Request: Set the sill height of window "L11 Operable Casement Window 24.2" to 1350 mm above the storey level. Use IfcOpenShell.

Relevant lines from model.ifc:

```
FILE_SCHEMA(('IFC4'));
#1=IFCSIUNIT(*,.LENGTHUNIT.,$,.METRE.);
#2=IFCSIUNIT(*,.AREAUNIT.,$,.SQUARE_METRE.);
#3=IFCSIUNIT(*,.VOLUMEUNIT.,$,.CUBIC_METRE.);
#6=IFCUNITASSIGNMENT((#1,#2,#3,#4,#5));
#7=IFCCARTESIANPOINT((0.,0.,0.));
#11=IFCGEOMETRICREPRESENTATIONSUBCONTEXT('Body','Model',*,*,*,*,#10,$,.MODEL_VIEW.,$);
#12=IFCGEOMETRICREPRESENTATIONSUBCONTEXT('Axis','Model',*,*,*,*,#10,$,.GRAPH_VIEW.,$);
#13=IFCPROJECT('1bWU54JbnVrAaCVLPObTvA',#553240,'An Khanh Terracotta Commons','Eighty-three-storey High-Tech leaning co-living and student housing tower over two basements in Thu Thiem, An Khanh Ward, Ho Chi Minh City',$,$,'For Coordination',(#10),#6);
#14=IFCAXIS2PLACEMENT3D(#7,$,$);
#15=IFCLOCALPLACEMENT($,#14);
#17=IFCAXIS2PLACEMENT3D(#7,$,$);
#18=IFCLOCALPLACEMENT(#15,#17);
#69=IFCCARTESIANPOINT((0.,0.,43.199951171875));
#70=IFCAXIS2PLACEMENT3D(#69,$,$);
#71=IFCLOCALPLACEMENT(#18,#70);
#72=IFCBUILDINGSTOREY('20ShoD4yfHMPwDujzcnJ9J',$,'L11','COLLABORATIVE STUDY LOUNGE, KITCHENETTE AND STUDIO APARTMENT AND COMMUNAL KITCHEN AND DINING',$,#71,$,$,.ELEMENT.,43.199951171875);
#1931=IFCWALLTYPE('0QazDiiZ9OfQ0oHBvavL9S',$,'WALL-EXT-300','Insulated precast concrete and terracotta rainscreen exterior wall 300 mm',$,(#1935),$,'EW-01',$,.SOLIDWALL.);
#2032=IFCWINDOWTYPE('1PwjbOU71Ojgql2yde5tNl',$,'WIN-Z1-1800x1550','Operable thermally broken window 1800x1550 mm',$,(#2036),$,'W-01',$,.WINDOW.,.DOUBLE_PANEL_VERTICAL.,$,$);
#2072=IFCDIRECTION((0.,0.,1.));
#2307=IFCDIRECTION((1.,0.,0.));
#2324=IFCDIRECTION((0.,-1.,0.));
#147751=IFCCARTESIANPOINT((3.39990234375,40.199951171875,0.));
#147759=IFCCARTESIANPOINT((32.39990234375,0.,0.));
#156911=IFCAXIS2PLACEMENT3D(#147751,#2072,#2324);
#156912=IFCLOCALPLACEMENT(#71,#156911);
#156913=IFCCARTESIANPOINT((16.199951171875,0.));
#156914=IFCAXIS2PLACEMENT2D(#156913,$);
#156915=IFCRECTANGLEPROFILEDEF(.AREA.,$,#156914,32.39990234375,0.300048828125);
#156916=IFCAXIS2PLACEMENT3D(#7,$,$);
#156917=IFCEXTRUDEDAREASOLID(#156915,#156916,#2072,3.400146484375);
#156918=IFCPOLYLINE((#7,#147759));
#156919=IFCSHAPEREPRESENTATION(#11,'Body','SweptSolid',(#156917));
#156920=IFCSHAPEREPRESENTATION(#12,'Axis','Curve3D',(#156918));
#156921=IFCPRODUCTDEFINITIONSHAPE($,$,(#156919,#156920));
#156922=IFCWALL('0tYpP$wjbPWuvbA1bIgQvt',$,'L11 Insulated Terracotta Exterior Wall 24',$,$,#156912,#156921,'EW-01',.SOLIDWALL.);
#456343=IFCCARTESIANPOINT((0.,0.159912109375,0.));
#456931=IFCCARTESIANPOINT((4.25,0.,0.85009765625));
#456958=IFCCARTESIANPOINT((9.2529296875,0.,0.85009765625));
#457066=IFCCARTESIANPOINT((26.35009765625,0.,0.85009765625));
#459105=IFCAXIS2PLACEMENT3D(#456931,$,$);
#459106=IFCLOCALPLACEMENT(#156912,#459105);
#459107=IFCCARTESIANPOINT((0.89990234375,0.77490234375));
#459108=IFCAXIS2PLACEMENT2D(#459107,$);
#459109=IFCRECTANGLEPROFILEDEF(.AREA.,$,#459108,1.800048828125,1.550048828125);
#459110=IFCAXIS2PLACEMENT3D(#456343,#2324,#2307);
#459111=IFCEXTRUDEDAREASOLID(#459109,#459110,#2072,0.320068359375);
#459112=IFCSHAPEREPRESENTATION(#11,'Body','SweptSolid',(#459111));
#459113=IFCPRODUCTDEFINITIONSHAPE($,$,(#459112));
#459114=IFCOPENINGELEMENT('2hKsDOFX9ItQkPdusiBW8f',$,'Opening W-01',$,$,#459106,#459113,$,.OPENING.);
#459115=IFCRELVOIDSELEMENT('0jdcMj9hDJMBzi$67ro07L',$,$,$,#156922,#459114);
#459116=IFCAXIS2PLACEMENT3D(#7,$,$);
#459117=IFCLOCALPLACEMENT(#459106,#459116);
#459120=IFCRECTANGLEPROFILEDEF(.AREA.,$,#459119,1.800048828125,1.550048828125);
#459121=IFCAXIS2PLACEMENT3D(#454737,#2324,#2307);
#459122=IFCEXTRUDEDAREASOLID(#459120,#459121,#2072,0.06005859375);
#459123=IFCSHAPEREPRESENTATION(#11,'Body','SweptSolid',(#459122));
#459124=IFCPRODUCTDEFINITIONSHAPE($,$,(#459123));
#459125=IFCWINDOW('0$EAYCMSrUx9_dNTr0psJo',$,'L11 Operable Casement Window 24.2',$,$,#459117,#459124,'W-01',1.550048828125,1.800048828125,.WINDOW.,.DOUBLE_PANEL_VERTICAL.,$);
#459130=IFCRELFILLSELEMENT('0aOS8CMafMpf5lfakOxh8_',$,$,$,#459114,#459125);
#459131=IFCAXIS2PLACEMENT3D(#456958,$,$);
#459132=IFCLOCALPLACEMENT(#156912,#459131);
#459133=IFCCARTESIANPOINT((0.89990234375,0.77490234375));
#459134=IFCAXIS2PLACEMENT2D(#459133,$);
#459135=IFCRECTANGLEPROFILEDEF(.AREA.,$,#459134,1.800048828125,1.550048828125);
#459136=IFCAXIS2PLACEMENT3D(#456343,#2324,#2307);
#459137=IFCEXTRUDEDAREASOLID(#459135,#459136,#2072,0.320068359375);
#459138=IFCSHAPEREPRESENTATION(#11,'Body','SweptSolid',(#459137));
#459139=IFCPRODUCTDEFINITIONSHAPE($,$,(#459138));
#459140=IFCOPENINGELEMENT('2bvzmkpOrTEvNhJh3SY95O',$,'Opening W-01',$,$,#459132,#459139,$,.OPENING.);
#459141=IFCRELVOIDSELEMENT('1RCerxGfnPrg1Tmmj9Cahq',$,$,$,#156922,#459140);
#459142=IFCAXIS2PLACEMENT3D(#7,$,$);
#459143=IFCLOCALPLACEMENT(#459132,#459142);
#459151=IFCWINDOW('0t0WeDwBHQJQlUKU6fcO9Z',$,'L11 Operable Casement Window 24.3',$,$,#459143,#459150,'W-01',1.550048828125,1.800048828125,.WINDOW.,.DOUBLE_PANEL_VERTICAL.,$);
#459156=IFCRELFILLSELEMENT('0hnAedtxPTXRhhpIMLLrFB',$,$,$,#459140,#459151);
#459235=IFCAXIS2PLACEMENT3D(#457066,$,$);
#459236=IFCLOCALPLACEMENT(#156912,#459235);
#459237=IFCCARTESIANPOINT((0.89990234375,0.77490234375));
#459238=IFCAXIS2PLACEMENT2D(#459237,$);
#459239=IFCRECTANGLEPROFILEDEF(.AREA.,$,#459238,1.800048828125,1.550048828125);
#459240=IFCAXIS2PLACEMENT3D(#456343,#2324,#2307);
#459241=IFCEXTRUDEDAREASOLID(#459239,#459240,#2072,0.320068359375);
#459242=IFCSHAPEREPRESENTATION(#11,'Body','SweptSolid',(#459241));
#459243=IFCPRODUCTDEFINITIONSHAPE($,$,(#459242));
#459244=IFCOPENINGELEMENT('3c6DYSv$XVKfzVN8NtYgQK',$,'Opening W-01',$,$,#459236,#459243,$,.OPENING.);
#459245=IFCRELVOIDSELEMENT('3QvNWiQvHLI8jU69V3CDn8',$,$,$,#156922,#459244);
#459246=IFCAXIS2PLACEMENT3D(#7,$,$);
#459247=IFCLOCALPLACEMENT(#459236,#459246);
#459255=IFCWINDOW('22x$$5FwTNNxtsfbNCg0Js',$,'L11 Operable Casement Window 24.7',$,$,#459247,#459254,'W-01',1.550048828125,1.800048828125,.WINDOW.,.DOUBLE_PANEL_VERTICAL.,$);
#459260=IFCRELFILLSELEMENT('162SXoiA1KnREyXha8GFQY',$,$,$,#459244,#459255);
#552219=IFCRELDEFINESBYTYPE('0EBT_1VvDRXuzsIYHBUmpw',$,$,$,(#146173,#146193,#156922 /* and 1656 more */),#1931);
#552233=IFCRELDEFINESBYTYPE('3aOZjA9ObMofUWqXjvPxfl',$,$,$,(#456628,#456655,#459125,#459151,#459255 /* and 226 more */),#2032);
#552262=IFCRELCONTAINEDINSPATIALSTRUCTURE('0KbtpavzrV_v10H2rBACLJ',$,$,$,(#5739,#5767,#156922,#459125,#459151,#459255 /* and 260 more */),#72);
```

```python
import numpy as np
import ifcopenshell
import ifcopenshell.api.geometry
import ifcopenshell.geom
import ifcopenshell.util.element
import ifcopenshell.util.placement
import ifcopenshell.util.shape
import ifcopenshell.util.unit

model = ifcopenshell.open("model.ifc")
unit_scale = ifcopenshell.util.unit.calculate_unit_scale(model)

window = model.by_guid("0$EAYCMSrUx9_dNTr0psJo")
opening = window.FillsVoids[0].RelatingOpeningElement
storey = ifcopenshell.util.element.get_container(window, ifc_class="IfcBuildingStorey")
level = ifcopenshell.util.placement.get_local_placement(storey.ObjectPlacement)[2, 3]

# The opening's origin need not be at the sill, so measure its lowest point.
shape = ifcopenshell.geom.create_shape(ifcopenshell.geom.settings(), opening)
bottom = ifcopenshell.util.shape.get_shape_bottom_elevation(shape, shape.geometry) / unit_scale
dz = level + 1.35 - bottom

shift = np.array([0.0, 0.0, dz])
# The window is placed relative to its opening, so it follows when the opening moves.
matrix = ifcopenshell.util.placement.get_local_placement(opening.ObjectPlacement)
matrix[:3, 3] += shift
ifcopenshell.api.geometry.edit_object_placement(
    model, product=opening, matrix=matrix, is_si=False, should_transform_children=True
)

print(f"moved by {dz * unit_scale:+.3f} m")

model.write("model_rev.ifc")
```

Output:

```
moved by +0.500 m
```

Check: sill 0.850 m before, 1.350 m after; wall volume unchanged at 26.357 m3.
